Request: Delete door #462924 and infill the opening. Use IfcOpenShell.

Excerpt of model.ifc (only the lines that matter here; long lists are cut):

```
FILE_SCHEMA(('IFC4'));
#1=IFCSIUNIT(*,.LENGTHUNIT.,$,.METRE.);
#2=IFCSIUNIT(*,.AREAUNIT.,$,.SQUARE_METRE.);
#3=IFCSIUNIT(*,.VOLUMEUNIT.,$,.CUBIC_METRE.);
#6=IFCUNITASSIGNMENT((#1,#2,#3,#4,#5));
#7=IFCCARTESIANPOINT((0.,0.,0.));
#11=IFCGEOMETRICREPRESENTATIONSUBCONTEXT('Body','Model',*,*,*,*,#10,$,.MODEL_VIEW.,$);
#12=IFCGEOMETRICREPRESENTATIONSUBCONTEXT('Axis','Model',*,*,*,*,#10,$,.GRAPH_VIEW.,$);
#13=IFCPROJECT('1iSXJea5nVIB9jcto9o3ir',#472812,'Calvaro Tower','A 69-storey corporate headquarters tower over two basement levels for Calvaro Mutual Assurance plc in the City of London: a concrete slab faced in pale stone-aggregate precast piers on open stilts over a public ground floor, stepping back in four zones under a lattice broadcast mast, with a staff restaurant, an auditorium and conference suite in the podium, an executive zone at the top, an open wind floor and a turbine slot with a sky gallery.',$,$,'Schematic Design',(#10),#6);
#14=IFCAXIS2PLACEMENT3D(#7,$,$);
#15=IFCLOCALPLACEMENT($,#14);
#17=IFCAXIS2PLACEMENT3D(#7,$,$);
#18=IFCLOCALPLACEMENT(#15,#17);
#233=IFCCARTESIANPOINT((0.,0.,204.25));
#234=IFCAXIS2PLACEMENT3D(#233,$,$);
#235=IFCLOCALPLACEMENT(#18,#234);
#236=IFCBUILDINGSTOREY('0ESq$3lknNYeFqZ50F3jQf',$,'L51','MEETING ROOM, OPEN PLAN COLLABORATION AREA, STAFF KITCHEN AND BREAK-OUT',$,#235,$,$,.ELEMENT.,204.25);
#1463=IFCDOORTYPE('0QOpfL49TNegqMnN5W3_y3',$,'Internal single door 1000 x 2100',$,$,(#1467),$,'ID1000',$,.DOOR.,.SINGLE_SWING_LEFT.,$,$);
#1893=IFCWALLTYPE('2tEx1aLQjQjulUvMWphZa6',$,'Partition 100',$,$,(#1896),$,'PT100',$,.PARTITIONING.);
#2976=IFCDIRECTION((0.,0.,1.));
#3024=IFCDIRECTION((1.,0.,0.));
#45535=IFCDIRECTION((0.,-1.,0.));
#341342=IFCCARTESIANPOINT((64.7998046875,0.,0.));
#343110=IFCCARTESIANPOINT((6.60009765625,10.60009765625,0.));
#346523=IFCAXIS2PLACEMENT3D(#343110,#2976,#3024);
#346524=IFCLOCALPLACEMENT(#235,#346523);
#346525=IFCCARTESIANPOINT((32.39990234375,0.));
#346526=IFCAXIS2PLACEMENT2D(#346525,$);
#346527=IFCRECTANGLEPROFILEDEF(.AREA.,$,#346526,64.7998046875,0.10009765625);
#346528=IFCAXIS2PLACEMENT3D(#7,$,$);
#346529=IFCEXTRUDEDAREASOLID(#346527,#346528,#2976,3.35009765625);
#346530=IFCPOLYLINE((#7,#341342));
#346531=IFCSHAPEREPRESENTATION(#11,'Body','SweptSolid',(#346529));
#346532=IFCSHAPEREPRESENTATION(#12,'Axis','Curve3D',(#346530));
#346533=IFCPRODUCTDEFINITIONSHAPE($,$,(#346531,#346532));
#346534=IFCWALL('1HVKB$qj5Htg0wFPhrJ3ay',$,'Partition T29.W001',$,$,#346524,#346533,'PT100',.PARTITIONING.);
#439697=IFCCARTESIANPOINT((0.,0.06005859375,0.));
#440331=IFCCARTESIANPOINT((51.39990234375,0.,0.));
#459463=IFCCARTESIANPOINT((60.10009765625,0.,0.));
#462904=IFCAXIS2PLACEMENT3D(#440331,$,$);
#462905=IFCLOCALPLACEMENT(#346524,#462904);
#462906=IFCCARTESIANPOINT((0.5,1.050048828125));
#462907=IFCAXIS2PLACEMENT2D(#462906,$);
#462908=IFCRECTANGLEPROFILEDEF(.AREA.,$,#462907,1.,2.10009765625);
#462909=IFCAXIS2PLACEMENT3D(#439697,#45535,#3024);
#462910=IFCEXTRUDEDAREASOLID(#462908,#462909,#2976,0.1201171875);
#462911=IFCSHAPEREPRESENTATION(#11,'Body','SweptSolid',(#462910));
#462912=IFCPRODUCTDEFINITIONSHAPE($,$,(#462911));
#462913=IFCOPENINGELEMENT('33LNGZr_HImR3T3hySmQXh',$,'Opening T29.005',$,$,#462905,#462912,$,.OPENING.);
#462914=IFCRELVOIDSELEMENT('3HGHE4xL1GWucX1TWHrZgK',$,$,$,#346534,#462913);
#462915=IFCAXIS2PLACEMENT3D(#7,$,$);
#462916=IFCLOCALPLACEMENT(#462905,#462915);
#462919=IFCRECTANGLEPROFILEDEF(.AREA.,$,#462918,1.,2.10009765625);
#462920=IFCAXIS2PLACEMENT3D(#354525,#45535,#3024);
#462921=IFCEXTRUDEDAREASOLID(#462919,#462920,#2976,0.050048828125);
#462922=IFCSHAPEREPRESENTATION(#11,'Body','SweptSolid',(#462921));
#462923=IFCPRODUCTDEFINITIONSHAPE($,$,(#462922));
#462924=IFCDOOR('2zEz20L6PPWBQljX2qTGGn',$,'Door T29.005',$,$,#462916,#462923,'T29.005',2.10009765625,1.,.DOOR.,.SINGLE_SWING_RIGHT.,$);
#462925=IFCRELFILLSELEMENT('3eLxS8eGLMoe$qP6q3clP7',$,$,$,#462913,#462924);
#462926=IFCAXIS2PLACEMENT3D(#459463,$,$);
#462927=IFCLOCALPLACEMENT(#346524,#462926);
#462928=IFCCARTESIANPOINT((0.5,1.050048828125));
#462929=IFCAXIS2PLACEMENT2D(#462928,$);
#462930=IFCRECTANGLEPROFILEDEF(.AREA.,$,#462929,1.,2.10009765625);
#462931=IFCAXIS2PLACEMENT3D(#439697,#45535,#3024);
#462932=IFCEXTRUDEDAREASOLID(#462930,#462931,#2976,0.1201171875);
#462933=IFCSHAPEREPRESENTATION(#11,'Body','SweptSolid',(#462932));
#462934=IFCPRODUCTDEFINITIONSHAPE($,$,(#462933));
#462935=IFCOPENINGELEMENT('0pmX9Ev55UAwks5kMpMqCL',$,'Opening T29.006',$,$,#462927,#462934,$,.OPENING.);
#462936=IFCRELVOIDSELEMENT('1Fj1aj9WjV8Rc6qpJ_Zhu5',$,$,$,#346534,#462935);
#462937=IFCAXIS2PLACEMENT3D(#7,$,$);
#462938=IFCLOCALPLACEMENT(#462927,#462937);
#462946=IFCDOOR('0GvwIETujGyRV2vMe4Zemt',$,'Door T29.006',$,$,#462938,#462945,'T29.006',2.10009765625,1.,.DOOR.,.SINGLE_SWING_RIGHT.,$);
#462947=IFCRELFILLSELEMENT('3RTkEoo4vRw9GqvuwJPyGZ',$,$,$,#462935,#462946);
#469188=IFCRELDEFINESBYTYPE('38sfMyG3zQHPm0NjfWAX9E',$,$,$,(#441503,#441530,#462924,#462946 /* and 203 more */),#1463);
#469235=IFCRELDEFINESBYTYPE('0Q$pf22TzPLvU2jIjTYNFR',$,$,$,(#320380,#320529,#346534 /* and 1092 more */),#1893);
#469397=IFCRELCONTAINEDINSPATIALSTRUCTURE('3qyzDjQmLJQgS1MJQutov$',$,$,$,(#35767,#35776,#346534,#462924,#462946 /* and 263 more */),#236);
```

```python
import ifcopenshell
import ifcopenshell.api.feature
import ifcopenshell.api.root
import ifcopenshell.geom
import ifcopenshell.util.shape

model = ifcopenshell.open("model.ifc")
settings = ifcopenshell.geom.settings()


def volume(element):
    """Net volume in cubic metres, openings subtracted."""
    shape = ifcopenshell.geom.create_shape(settings, element)
    return ifcopenshell.util.shape.get_volume(shape.geometry)


door = model.by_guid("2zEz20L6PPWBQljX2qTGGn")
opening = door.FillsVoids[0].RelatingOpeningElement
wall = opening.VoidsElements[0].RelatingBuildingElement
before = volume(wall)

ifcopenshell.api.root.remove_product(model, product=door)
ifcopenshell.api.feature.remove_feature(model, feature=opening)

after = volume(wall)

print(f"wall volume {before:.3f} -> {after:.3f} m3")

model.write("model-out.ifc")
```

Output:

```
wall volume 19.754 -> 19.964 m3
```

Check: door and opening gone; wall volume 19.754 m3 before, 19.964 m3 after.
